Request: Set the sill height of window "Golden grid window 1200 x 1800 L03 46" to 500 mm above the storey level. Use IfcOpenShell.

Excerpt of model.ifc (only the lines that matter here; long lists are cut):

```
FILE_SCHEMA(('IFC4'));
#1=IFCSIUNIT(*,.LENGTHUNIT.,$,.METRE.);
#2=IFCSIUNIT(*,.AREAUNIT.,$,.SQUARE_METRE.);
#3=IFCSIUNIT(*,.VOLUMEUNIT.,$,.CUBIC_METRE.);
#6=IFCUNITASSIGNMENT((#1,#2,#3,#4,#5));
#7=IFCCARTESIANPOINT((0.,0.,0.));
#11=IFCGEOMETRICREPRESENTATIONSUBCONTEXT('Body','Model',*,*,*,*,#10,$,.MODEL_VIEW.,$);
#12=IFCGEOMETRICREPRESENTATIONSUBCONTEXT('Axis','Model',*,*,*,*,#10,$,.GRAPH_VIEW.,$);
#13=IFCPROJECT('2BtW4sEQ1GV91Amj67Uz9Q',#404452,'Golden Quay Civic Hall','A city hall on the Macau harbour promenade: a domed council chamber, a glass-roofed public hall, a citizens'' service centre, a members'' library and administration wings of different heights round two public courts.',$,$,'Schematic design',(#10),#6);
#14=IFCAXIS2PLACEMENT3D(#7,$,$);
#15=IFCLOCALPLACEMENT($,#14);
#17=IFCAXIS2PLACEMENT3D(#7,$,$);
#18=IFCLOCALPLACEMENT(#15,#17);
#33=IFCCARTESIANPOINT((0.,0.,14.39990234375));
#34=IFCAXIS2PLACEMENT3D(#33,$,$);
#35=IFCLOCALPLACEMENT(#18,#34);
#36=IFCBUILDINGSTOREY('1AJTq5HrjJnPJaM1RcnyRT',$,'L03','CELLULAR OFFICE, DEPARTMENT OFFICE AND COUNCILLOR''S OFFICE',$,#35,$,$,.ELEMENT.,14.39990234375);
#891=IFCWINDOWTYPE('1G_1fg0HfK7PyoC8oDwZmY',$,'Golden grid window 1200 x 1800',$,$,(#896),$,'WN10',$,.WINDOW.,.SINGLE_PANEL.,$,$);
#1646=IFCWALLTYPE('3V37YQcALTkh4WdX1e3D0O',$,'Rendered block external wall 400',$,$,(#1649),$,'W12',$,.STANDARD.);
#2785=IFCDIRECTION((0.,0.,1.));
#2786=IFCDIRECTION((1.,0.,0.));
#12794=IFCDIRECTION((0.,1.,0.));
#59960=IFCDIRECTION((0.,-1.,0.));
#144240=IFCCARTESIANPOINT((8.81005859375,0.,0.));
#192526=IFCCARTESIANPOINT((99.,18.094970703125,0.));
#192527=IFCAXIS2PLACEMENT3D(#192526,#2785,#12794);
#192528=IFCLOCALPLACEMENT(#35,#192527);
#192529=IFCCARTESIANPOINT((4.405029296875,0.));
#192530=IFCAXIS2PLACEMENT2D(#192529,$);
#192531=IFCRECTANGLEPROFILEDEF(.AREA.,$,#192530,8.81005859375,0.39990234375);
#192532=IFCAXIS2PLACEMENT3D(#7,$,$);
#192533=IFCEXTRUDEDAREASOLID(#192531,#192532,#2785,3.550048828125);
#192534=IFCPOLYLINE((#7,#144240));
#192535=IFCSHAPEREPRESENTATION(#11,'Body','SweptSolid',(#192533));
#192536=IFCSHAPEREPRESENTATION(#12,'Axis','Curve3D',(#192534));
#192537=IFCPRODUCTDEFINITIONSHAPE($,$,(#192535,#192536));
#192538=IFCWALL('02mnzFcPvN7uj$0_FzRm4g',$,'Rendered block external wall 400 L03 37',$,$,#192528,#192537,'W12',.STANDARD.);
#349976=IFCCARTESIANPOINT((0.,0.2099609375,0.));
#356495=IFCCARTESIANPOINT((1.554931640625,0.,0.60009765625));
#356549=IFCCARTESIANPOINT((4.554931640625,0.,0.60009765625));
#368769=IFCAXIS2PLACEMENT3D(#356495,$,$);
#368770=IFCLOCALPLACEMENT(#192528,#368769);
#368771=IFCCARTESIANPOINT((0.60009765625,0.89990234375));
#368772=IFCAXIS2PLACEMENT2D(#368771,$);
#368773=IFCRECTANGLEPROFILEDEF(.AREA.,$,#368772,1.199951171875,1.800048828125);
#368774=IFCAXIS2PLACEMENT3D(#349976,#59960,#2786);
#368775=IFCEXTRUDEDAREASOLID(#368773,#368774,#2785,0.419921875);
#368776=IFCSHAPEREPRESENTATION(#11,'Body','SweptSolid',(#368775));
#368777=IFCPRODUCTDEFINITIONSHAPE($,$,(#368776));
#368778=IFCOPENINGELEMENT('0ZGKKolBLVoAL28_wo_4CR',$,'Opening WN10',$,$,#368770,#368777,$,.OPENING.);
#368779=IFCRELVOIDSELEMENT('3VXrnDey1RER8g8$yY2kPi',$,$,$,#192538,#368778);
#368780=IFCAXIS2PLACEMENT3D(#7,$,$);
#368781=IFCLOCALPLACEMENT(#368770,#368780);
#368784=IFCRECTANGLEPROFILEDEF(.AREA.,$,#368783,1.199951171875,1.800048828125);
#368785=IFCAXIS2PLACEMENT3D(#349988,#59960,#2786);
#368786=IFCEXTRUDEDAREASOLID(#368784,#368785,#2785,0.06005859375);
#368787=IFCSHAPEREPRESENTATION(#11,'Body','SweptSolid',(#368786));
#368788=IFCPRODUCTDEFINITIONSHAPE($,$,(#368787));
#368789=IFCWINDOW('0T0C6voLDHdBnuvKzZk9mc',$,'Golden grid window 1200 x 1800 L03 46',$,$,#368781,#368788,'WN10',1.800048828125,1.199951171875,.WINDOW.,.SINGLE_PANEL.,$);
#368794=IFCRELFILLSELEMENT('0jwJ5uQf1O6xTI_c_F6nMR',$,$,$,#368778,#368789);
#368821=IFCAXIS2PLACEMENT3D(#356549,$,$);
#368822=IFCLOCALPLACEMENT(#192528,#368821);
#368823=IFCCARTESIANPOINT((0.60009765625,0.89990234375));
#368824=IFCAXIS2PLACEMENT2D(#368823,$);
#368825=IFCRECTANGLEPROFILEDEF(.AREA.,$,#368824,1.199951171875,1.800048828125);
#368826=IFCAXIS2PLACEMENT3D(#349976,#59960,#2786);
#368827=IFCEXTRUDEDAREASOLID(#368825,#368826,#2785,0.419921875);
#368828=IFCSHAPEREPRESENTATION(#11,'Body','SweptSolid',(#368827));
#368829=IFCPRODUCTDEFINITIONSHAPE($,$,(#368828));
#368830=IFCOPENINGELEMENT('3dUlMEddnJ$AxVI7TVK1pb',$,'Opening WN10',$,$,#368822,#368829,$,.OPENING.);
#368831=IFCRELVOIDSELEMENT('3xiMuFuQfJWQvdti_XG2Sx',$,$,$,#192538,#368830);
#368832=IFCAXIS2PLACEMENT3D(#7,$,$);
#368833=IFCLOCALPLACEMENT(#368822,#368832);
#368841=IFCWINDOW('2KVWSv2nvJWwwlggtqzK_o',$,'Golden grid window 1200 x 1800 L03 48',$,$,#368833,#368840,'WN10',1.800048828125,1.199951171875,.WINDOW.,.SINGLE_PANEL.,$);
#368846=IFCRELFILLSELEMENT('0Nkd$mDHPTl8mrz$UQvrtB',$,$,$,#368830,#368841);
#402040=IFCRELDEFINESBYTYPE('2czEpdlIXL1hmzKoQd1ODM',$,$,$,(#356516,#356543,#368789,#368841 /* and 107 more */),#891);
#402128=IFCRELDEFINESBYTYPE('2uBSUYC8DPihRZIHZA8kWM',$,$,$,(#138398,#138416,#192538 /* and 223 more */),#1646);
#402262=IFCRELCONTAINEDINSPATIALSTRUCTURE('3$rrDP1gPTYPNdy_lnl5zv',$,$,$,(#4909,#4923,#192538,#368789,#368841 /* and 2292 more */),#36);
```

```python
import numpy as np
import ifcopenshell
import ifcopenshell.api.geometry
import ifcopenshell.geom
import ifcopenshell.util.element
import ifcopenshell.util.placement
import ifcopenshell.util.shape
import ifcopenshell.util.unit

model = ifcopenshell.open("model.ifc")
unit_scale = ifcopenshell.util.unit.calculate_unit_scale(model)

window = model.by_guid("0T0C6voLDHdBnuvKzZk9mc")
opening = window.FillsVoids[0].RelatingOpeningElement
storey = ifcopenshell.util.element.get_container(window, ifc_class="IfcBuildingStorey")
level = ifcopenshell.util.placement.get_local_placement(storey.ObjectPlacement)[2, 3]

# The opening's origin need not be at the sill, so measure its lowest point.
shape = ifcopenshell.geom.create_shape(ifcopenshell.geom.settings(), opening)
bottom = ifcopenshell.util.shape.get_shape_bottom_elevation(shape, shape.geometry) / unit_scale
dz = level + 0.5 - bottom

shift = np.array([0.0, 0.0, dz])
# The window is placed relative to its opening, so it follows when the opening moves.
matrix = ifcopenshell.util.placement.get_local_placement(opening.ObjectPlacement)
matrix[:3, 3] += shift
ifcopenshell.api.geometry.edit_object_placement(
    model, product=opening, matrix=matrix, is_si=False, should_transform_children=True
)

print(f"moved by {dz * unit_scale:+.3f} m")

model.write("model-out.ifc")
```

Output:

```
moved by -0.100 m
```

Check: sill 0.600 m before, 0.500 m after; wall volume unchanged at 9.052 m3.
